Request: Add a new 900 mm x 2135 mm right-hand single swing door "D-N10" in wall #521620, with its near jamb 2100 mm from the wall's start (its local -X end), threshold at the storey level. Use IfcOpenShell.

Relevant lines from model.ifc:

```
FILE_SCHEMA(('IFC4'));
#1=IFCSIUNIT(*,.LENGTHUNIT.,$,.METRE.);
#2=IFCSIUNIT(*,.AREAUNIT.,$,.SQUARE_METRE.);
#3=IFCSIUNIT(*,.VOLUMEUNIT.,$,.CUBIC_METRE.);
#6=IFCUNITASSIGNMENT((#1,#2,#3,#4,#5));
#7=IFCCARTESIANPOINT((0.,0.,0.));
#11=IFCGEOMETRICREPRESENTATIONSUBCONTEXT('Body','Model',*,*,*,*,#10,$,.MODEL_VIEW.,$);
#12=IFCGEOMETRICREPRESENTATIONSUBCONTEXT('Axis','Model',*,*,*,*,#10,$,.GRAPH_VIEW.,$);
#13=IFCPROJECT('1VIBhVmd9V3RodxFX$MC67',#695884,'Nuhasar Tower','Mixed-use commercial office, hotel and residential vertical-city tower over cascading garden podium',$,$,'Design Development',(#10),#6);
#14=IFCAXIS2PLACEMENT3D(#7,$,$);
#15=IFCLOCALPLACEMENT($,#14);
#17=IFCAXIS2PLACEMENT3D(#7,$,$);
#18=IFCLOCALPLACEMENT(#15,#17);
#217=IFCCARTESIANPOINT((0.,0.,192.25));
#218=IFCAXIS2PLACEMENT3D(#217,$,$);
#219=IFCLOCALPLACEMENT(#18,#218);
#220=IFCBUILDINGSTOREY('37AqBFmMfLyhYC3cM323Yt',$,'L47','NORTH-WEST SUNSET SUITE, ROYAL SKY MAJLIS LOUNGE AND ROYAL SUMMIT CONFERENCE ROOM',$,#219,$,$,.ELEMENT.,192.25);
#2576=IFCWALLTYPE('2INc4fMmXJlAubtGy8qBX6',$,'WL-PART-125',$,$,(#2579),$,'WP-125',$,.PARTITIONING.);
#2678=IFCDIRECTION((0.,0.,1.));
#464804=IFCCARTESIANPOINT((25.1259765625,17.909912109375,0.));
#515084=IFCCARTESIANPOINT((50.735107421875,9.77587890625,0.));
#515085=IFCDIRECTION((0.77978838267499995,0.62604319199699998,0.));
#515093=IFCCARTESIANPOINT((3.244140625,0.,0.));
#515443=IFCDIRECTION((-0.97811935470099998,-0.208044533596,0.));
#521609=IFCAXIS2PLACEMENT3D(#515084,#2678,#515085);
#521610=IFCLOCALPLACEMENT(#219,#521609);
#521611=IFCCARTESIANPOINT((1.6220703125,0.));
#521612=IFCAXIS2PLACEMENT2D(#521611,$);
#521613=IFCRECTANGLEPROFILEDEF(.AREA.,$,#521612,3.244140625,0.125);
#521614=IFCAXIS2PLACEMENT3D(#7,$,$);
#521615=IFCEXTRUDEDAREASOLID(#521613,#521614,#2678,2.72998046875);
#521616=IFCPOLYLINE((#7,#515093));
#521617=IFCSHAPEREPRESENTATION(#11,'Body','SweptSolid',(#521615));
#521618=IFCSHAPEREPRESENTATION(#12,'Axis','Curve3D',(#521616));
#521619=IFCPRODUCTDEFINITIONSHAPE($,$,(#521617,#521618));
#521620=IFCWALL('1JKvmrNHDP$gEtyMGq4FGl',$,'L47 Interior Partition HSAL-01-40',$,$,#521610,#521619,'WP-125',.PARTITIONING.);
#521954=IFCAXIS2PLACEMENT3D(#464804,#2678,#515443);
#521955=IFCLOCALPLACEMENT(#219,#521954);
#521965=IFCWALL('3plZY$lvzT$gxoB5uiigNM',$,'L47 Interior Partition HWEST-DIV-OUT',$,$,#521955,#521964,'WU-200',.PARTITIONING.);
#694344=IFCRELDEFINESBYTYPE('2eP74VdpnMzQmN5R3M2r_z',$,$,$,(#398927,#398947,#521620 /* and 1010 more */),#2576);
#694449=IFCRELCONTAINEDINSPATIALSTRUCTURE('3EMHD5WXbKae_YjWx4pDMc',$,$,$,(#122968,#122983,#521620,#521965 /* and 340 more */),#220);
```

```python
import numpy as np
import ifcopenshell
import ifcopenshell.api.feature
import ifcopenshell.api.geometry
import ifcopenshell.api.root
import ifcopenshell.api.spatial
import ifcopenshell.geom
import ifcopenshell.util.element
import ifcopenshell.util.placement
import ifcopenshell.util.representation
import ifcopenshell.util.shape
import ifcopenshell.util.unit

model = ifcopenshell.open("model.ifc")
unit_scale = ifcopenshell.util.unit.calculate_unit_scale(model)
settings = ifcopenshell.geom.settings()


def volume(element):
    """Net volume in cubic metres, openings subtracted."""
    shape = ifcopenshell.geom.create_shape(settings, element)
    return ifcopenshell.util.shape.get_volume(shape.geometry)


wall = model.by_guid("1JKvmrNHDP$gEtyMGq4FGl")
storey = ifcopenshell.util.element.get_container(wall, ifc_class="IfcBuildingStorey")
context = ifcopenshell.util.representation.get_context(model, "Model", "Body", "MODEL_VIEW")
before = volume(wall)

width, height, from_end, sill = 0.9, 2.135, 2.1, 0.0  # metres

# The wall runs along its own X axis, and the end named is its -X end.
wall_shape = ifcopenshell.geom.create_shape(settings, wall)
x, y, z = ifcopenshell.util.shape.get_vertices(wall_shape.geometry).T
start = x.min() + from_end
face, thickness = float(y.min()), float(y.max() - y.min())
wall_matrix = ifcopenshell.util.placement.get_local_placement(wall.ObjectPlacement)
level = ifcopenshell.util.placement.get_local_placement(storey.ObjectPlacement)[2, 3]


def in_wall(x, y):
    """Placement at x, y metres in the wall's axes, at sill height."""
    matrix = wall_matrix.copy()
    matrix[:, 3] = wall_matrix @ np.array([x / unit_scale, y / unit_scale, 0.0, 1.0])
    matrix[2, 3] = level + sill / unit_scale
    return matrix


# Opening: a box that overshoots both wall faces by 50 mm.
opening = ifcopenshell.api.root.create_entity(model, ifc_class="IfcOpeningElement", predefined_type="OPENING")
box = ifcopenshell.api.geometry.add_wall_representation(
    model, context=context, length=width, height=height, thickness=thickness + 0.1
)
ifcopenshell.api.geometry.assign_representation(model, product=opening, representation=box)
ifcopenshell.api.geometry.edit_object_placement(model, product=opening, matrix=in_wall(start, face - 0.05), is_si=False)
ifcopenshell.api.feature.add_feature(model, feature=opening, element=wall)

door = ifcopenshell.api.root.create_entity(model, ifc_class="IfcDoor", name="D-N10", predefined_type="DOOR")
door.OverallWidth, door.OverallHeight = width / unit_scale, height / unit_scale
door.OperationType = "SINGLE_SWING_RIGHT"
body = ifcopenshell.api.geometry.add_door_representation(
    model,
    context=context,
    overall_width=door.OverallWidth,
    overall_height=door.OverallHeight,
    operation_type="SINGLE_SWING_RIGHT",
    lining_properties={"LiningDepth": thickness / unit_scale, "ThresholdDepth": thickness / unit_scale},
)
ifcopenshell.api.geometry.assign_representation(model, product=door, representation=body)
ifcopenshell.api.spatial.assign_container(model, products=[door], relating_structure=storey)
ifcopenshell.api.feature.add_filling(model, opening=opening, element=door)

# The lining spans the wall, so the door starts at the wall face.
ifcopenshell.api.geometry.edit_object_placement(model, product=door, matrix=in_wall(start, face), is_si=False)

after = volume(wall)

print(f"wall volume {before:.3f} -> {after:.3f} m3")

model.write("model_v2.ifc")
```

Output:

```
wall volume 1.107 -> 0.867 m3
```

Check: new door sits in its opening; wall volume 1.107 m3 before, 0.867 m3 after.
